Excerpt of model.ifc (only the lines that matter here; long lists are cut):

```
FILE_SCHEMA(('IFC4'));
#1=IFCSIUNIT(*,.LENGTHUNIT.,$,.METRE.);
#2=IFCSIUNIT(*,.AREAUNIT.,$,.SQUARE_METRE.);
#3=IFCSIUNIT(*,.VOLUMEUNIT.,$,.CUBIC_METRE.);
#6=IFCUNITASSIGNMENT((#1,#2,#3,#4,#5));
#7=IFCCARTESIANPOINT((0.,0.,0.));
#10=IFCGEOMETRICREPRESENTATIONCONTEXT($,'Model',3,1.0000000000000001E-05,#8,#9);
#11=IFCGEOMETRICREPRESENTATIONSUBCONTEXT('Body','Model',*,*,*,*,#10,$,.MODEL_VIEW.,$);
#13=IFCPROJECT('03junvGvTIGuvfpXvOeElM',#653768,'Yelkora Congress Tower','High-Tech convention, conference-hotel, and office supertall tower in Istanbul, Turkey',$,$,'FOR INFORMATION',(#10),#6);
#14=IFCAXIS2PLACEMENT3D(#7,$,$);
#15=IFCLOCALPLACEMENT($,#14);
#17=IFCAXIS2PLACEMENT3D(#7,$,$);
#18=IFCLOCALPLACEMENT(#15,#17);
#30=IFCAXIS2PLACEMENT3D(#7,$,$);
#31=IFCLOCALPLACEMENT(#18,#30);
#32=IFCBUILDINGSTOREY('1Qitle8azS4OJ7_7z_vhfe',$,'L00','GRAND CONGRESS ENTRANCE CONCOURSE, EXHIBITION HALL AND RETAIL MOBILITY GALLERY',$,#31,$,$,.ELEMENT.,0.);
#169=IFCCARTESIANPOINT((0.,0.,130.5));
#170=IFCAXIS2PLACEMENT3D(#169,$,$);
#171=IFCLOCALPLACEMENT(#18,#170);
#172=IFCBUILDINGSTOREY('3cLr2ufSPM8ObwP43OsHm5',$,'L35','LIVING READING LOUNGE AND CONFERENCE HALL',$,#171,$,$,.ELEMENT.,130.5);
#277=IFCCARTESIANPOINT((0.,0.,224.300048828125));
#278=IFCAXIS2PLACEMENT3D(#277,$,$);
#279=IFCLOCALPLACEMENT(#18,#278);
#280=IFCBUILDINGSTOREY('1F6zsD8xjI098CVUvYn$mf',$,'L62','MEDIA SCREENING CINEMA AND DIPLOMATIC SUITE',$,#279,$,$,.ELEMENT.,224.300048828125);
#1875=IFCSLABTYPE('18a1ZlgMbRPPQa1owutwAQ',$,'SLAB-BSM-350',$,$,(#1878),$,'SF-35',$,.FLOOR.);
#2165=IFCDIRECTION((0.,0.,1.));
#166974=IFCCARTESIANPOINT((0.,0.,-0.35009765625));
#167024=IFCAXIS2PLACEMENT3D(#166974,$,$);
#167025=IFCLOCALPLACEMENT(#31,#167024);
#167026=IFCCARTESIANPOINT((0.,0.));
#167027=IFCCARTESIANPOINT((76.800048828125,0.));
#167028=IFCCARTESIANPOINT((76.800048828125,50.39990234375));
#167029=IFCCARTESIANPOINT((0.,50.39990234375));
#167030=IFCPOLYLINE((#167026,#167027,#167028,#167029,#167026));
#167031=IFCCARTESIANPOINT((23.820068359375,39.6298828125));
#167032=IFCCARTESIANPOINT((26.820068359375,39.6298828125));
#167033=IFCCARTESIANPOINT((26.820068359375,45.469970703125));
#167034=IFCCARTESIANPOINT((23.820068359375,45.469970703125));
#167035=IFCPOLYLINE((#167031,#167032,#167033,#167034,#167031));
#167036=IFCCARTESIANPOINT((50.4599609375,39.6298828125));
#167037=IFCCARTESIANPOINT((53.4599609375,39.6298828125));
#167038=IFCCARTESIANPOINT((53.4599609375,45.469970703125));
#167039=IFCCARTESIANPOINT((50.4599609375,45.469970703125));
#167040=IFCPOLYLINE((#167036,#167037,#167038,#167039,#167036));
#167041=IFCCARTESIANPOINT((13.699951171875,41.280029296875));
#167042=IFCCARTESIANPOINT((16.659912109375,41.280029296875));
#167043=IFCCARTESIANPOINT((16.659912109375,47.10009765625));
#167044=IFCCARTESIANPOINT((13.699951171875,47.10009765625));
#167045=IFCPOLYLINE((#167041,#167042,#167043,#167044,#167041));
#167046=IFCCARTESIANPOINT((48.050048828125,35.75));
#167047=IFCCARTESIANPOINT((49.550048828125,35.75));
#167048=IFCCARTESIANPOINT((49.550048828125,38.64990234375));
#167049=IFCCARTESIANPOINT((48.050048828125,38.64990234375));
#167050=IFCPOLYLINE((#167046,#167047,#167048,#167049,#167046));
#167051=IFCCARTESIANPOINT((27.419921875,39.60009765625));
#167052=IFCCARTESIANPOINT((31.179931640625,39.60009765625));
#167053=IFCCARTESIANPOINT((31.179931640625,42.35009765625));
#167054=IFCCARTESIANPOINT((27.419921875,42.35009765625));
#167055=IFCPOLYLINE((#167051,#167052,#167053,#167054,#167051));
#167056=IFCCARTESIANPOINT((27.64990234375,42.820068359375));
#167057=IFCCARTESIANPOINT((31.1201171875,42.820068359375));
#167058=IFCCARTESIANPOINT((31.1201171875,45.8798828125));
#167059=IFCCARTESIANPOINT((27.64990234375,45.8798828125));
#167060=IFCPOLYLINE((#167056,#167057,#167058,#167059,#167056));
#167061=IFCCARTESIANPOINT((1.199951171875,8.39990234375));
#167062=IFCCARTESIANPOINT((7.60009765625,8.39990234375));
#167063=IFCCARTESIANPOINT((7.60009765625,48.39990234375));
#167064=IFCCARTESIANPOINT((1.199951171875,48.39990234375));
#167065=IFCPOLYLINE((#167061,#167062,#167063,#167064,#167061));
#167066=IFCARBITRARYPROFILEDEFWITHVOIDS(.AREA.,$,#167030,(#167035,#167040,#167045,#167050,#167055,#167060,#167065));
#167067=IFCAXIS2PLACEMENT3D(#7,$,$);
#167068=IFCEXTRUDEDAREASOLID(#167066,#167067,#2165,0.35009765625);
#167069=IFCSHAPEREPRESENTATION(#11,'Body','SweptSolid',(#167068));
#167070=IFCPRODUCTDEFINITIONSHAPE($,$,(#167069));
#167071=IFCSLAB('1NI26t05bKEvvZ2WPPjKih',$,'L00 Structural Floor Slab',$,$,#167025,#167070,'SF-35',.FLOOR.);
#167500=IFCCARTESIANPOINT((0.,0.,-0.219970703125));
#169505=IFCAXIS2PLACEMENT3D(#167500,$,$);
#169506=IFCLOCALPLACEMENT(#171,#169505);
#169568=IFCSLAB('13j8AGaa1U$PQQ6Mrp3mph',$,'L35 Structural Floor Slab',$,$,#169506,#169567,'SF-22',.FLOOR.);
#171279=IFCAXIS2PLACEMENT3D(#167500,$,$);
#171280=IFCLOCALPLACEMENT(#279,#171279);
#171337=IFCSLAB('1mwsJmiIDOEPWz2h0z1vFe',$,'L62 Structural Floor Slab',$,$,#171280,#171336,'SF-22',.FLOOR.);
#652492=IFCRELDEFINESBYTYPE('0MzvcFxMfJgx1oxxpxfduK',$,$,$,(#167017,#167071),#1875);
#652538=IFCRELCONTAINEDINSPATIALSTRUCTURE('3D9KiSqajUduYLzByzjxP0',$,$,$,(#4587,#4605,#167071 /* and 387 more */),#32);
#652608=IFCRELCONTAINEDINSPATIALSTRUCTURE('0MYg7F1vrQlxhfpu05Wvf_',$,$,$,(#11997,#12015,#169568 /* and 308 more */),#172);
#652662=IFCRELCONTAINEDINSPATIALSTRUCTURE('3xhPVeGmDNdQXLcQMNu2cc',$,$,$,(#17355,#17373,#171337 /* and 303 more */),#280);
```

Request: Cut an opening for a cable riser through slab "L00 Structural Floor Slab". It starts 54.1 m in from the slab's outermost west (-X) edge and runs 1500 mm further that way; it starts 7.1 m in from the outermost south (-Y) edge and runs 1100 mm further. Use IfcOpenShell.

```python
import numpy as np
import ifcopenshell
import ifcopenshell.api.feature
import ifcopenshell.api.geometry
import ifcopenshell.api.root
import ifcopenshell.geom
import ifcopenshell.util.placement
import ifcopenshell.util.representation
import ifcopenshell.util.shape
import ifcopenshell.util.unit

model = ifcopenshell.open("model.ifc")
unit_scale = ifcopenshell.util.unit.calculate_unit_scale(model)
settings = ifcopenshell.geom.settings()


def volume(element):
    """Net volume in cubic metres, openings subtracted."""
    shape = ifcopenshell.geom.create_shape(settings, element)
    return ifcopenshell.util.shape.get_volume(shape.geometry)


slab = model.by_guid("1NI26t05bKEvvZ2WPPjKih")
before = volume(slab)

# Extent in the slab's own axes, in metres. The edges named are its -X and -Y sides.
slab_shape = ifcopenshell.geom.create_shape(settings, slab)
vertices = ifcopenshell.util.shape.get_vertices(slab_shape.geometry)
x_min, y_min, bottom = vertices.min(axis=0)
top = vertices[:, 2].max()

opening = ifcopenshell.api.root.create_entity(model, ifc_class="IfcOpeningElement", name="Cable riser opening", predefined_type="OPENING")
context = ifcopenshell.util.representation.get_context(model, "Model", "Body", "MODEL_VIEW")
width, depth = 1.5, 1.1
outline = [(0.0, 0.0), (width, 0.0), (width, depth), (0.0, depth), (0.0, 0.0)]
# Overshoot both faces by 50 mm so the cut is clean.
shape = ifcopenshell.api.geometry.add_slab_representation(
    model, context=context, depth=top - bottom + 0.1, polyline=outline
)
ifcopenshell.api.geometry.assign_representation(model, product=opening, representation=shape)

matrix = ifcopenshell.util.placement.get_local_placement(slab.ObjectPlacement)
matrix[:, 3] = matrix @ np.append(np.array([x_min + 54.1, y_min + 7.1, bottom - 0.05]) / unit_scale, 1.0)
ifcopenshell.api.geometry.edit_object_placement(model, product=opening, matrix=matrix, is_si=False)
ifcopenshell.api.feature.add_feature(model, feature=opening, element=slab)

after = volume(slab)

print(f"slab volume {before:.3f} -> {after:.3f} m3")

model.write("model_updated.ifc")
```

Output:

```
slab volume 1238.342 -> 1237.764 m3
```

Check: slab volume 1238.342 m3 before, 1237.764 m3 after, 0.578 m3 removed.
